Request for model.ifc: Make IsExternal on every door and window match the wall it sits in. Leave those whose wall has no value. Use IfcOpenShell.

First a look at what the model holds.

```python
import ifcopenshell
import ifcopenshell.util.element

model = ifcopenshell.open("model.ifc")
print(model.schema)
seen = {}
for e in model.by_type("IfcDoor") + model.by_type("IfcWindow"):
    if not e.FillsVoids:
        continue
    host = e.FillsVoids[0].RelatingOpeningElement.VoidsElements[0].RelatingBuildingElement
    own = ifcopenshell.util.element.get_pset(e, f"Pset_{e.is_a()[3:].removesuffix('StandardCase')}Common", "IsExternal")
    wall = ifcopenshell.util.element.get_pset(host, "Pset_WallCommon", "IsExternal")
    seen[e.is_a(), own, wall] = seen.get((e.is_a(), own, wall), 0) + 1
for (cls, own, wall), count in sorted(seen.items(), key=str):
    print(count, cls, "IsExternal:", own, "| host wall:", wall)
```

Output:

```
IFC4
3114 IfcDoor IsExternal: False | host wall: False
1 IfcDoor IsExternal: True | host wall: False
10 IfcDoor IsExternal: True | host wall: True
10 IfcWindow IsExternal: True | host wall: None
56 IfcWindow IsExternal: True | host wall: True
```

```python
import ifcopenshell
import ifcopenshell.api.pset
import ifcopenshell.util.element

model = ifcopenshell.open("model.ifc")

count = 0
for ifc_class, pset_name in (("IfcDoor", "Pset_DoorCommon"), ("IfcWindow", "Pset_WindowCommon")):
    for e in model.by_type(ifc_class):
        if not e.FillsVoids:
            continue
        host = e.FillsVoids[0].RelatingOpeningElement.VoidsElements[0].RelatingBuildingElement
        external = ifcopenshell.util.element.get_pset(host, "Pset_WallCommon", "IsExternal")
        if external is None or ifcopenshell.util.element.get_pset(e, pset_name, "IsExternal") == external:
            continue
        pset = ifcopenshell.api.pset.add_pset(model, product=e, name=pset_name)
        ifcopenshell.api.pset.edit_pset(model, pset=pset, properties={"IsExternal": external})
        count += 1

print(count, "updated")

model.write("model_updated.ifc")
```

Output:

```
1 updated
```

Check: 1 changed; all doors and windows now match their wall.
